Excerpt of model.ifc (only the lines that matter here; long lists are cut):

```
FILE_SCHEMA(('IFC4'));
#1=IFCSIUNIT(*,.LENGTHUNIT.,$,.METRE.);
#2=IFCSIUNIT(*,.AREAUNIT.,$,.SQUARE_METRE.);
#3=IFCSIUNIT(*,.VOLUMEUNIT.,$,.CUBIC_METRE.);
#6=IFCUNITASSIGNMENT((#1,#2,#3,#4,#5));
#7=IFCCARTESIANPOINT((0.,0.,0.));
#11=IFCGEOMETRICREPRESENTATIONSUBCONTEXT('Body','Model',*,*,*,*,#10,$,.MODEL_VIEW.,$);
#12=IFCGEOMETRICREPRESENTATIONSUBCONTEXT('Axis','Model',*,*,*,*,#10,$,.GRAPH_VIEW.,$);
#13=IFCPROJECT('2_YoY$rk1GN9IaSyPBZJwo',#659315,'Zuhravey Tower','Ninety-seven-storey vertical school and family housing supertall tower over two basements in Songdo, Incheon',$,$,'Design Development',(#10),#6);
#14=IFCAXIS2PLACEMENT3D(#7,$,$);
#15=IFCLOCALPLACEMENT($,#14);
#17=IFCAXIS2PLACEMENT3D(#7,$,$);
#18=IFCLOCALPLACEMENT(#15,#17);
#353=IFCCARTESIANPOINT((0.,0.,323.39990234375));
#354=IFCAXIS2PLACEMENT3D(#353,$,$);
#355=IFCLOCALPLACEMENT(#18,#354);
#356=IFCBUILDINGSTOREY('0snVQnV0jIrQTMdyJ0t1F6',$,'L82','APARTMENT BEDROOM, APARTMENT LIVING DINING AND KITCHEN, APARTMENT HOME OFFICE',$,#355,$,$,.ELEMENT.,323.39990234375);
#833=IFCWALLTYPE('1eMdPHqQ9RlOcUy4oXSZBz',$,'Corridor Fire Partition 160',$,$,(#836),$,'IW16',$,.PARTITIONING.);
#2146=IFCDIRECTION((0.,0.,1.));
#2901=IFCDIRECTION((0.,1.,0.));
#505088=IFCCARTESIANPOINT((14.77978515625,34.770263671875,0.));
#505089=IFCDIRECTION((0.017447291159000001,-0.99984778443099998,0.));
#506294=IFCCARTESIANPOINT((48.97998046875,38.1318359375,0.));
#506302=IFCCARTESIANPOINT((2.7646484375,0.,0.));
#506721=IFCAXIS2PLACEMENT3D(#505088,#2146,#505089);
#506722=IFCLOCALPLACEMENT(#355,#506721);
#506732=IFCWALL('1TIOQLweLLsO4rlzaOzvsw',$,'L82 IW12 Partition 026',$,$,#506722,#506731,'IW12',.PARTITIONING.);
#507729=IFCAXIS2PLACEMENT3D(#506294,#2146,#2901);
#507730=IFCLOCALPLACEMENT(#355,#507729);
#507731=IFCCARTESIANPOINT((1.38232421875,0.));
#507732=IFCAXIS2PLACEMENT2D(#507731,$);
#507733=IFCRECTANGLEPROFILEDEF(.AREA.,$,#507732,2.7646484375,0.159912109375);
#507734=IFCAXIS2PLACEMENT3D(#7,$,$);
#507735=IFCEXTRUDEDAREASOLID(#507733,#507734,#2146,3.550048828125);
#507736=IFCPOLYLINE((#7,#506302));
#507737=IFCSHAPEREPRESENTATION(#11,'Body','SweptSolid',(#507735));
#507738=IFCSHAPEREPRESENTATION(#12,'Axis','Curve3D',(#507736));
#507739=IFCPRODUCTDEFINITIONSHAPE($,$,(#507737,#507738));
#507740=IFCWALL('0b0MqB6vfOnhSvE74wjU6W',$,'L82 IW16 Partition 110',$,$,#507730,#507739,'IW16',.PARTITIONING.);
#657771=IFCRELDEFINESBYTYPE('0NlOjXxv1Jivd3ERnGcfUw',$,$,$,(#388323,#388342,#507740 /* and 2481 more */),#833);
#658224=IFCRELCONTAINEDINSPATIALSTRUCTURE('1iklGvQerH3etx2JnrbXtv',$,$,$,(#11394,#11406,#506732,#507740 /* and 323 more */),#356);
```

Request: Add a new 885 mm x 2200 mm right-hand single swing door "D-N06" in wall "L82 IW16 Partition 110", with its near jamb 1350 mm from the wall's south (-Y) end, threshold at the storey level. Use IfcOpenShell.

```python
import numpy as np
import ifcopenshell
import ifcopenshell.api.feature
import ifcopenshell.api.geometry
import ifcopenshell.api.root
import ifcopenshell.api.spatial
import ifcopenshell.geom
import ifcopenshell.util.element
import ifcopenshell.util.placement
import ifcopenshell.util.representation
import ifcopenshell.util.shape
import ifcopenshell.util.unit

model = ifcopenshell.open("model.ifc")
unit_scale = ifcopenshell.util.unit.calculate_unit_scale(model)
settings = ifcopenshell.geom.settings()


def volume(element):
    """Net volume in cubic metres, openings subtracted."""
    shape = ifcopenshell.geom.create_shape(settings, element)
    return ifcopenshell.util.shape.get_volume(shape.geometry)


wall = model.by_guid("0b0MqB6vfOnhSvE74wjU6W")
storey = ifcopenshell.util.element.get_container(wall, ifc_class="IfcBuildingStorey")
context = ifcopenshell.util.representation.get_context(model, "Model", "Body", "MODEL_VIEW")
before = volume(wall)

width, height, from_end, sill = 0.885, 2.2, 1.35, 0.0  # metres

# The wall runs along its own X axis, and the end named is its -X end.
wall_shape = ifcopenshell.geom.create_shape(settings, wall)
x, y, z = ifcopenshell.util.shape.get_vertices(wall_shape.geometry).T
start = x.min() + from_end
face, thickness = float(y.min()), float(y.max() - y.min())
wall_matrix = ifcopenshell.util.placement.get_local_placement(wall.ObjectPlacement)
level = ifcopenshell.util.placement.get_local_placement(storey.ObjectPlacement)[2, 3]


def in_wall(x, y):
    """Placement at x, y metres in the wall's axes, at sill height."""
    matrix = wall_matrix.copy()
    matrix[:, 3] = wall_matrix @ np.array([x / unit_scale, y / unit_scale, 0.0, 1.0])
    matrix[2, 3] = level + sill / unit_scale
    return matrix


# Opening: a box that overshoots both wall faces by 50 mm.
opening = ifcopenshell.api.root.create_entity(model, ifc_class="IfcOpeningElement", predefined_type="OPENING")
box = ifcopenshell.api.geometry.add_wall_representation(
    model, context=context, length=width, height=height, thickness=thickness + 0.1
)
ifcopenshell.api.geometry.assign_representation(model, product=opening, representation=box)
ifcopenshell.api.geometry.edit_object_placement(model, product=opening, matrix=in_wall(start, face - 0.05), is_si=False)
ifcopenshell.api.feature.add_feature(model, feature=opening, element=wall)

door = ifcopenshell.api.root.create_entity(model, ifc_class="IfcDoor", name="D-N06", predefined_type="DOOR")
door.OverallWidth, door.OverallHeight = width / unit_scale, height / unit_scale
door.OperationType = "SINGLE_SWING_RIGHT"
body = ifcopenshell.api.geometry.add_door_representation(
    model,
    context=context,
    overall_width=door.OverallWidth,
    overall_height=door.OverallHeight,
    operation_type="SINGLE_SWING_RIGHT",
    lining_properties={"LiningDepth": thickness / unit_scale, "ThresholdDepth": thickness / unit_scale},
)
ifcopenshell.api.geometry.assign_representation(model, product=door, representation=body)
ifcopenshell.api.spatial.assign_container(model, products=[door], relating_structure=storey)
ifcopenshell.api.feature.add_filling(model, opening=opening, element=door)

# The lining spans the wall, so the door starts at the wall face.
ifcopenshell.api.geometry.edit_object_placement(model, product=door, matrix=in_wall(start, face), is_si=False)

after = volume(wall)

print(f"wall volume {before:.3f} -> {after:.3f} m3")

model.write("model_v2.ifc")
```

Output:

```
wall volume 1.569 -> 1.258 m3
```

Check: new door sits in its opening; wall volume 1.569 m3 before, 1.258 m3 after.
